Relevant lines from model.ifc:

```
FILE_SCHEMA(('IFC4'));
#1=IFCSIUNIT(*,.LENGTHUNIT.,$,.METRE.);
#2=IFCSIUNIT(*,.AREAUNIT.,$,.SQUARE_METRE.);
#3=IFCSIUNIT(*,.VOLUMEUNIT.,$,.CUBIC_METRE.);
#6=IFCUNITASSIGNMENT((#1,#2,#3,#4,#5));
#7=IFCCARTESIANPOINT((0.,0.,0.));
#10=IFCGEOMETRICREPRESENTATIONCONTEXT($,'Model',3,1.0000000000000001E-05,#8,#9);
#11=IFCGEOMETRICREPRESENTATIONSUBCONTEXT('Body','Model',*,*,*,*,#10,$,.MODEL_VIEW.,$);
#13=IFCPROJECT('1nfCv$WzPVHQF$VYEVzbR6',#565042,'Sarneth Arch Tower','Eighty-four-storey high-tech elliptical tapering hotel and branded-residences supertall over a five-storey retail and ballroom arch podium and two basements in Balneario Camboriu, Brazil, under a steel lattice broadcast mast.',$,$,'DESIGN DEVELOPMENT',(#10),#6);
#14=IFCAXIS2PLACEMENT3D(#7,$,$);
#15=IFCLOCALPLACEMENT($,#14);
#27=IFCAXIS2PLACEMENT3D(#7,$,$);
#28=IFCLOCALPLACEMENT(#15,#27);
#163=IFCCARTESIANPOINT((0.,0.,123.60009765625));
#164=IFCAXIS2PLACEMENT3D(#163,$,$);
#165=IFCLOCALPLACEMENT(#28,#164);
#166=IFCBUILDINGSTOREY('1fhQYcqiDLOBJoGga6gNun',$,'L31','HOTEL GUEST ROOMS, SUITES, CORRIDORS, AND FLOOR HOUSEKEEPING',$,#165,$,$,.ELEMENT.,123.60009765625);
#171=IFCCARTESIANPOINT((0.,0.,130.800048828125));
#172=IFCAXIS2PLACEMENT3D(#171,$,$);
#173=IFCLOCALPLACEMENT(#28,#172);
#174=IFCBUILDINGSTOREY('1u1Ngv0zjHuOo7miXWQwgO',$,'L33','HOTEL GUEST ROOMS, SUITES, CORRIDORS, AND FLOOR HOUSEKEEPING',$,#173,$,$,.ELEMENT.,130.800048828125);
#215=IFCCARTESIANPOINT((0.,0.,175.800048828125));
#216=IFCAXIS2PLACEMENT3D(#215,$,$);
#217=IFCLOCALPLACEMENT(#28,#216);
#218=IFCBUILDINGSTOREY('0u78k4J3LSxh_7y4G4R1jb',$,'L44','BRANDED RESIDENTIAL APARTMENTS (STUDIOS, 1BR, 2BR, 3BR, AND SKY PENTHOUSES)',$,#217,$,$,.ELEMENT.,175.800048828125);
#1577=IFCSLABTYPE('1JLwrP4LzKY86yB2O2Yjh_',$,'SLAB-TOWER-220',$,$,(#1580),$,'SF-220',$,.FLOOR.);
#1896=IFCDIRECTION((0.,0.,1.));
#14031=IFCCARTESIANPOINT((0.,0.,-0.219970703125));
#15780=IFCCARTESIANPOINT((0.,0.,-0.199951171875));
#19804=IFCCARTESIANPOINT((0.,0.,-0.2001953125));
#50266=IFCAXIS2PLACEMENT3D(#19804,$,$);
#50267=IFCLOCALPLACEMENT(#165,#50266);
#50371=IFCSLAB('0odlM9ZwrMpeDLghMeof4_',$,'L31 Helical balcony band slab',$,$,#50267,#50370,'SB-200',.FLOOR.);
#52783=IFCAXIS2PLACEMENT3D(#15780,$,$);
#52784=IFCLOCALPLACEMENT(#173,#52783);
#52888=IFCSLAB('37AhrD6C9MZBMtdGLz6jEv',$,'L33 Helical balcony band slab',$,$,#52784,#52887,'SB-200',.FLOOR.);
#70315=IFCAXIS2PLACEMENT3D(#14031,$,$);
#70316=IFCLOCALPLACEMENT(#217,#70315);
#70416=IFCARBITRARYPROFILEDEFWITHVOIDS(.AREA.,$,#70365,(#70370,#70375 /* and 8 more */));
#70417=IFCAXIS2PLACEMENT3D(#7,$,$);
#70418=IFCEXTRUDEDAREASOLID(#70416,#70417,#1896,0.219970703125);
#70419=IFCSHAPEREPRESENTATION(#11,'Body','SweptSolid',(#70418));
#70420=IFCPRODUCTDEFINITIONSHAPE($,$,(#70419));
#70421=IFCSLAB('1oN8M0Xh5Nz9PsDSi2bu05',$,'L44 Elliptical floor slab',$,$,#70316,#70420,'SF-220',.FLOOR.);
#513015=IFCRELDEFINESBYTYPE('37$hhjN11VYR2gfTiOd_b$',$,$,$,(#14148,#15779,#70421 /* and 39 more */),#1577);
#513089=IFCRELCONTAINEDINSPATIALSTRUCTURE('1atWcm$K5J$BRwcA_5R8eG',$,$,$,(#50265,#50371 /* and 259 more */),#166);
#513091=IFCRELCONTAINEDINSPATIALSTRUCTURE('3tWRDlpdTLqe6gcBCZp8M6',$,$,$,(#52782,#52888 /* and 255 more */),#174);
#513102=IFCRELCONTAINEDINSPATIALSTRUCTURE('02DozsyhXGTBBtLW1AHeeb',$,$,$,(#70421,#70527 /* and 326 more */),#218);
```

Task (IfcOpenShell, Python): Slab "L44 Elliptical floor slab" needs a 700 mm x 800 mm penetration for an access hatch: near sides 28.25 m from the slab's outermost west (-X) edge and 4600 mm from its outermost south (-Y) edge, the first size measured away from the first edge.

```python
import numpy as np
import ifcopenshell
import ifcopenshell.api.feature
import ifcopenshell.api.geometry
import ifcopenshell.api.root
import ifcopenshell.geom
import ifcopenshell.util.placement
import ifcopenshell.util.representation
import ifcopenshell.util.shape
import ifcopenshell.util.unit

model = ifcopenshell.open("model.ifc")
unit_scale = ifcopenshell.util.unit.calculate_unit_scale(model)
settings = ifcopenshell.geom.settings()


def volume(element):
    """Net volume in cubic metres, openings subtracted."""
    shape = ifcopenshell.geom.create_shape(settings, element)
    return ifcopenshell.util.shape.get_volume(shape.geometry)


slab = model.by_guid("1oN8M0Xh5Nz9PsDSi2bu05")
before = volume(slab)

# Extent in the slab's own axes, in metres. The edges named are its -X and -Y sides.
slab_shape = ifcopenshell.geom.create_shape(settings, slab)
vertices = ifcopenshell.util.shape.get_vertices(slab_shape.geometry)
x_min, y_min, bottom = vertices.min(axis=0)
top = vertices[:, 2].max()

opening = ifcopenshell.api.root.create_entity(model, ifc_class="IfcOpeningElement", name="Access hatch opening", predefined_type="OPENING")
context = ifcopenshell.util.representation.get_context(model, "Model", "Body", "MODEL_VIEW")
width, depth = 0.7, 0.8
outline = [(0.0, 0.0), (width, 0.0), (width, depth), (0.0, depth), (0.0, 0.0)]
# Overshoot both faces by 50 mm so the cut is clean.
shape = ifcopenshell.api.geometry.add_slab_representation(
    model, context=context, depth=top - bottom + 0.1, polyline=outline
)
ifcopenshell.api.geometry.assign_representation(model, product=opening, representation=shape)

matrix = ifcopenshell.util.placement.get_local_placement(slab.ObjectPlacement)
matrix[:, 3] = matrix @ np.append(np.array([x_min + 28.25, y_min + 4.6, bottom - 0.05]) / unit_scale, 1.0)
ifcopenshell.api.geometry.edit_object_placement(model, product=opening, matrix=matrix, is_si=False)
ifcopenshell.api.feature.add_feature(model, feature=opening, element=slab)

after = volume(slab)

print(f"slab volume {before:.3f} -> {after:.3f} m3")

model.write("model-out.ifc")
```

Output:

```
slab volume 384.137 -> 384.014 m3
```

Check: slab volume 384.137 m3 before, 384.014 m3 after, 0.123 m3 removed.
